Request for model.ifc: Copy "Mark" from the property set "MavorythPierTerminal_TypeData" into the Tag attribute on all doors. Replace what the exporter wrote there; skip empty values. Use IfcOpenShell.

First a look at what the model holds.

```python
import ifcopenshell
import ifcopenshell.util.element

model = ifcopenshell.open("model.ifc")
print(model.schema)
doors = model.by_type("IfcDoor")
print(len(doors), "doors")
for e in doors[:8]:
    source = ifcopenshell.util.element.get_pset(e, "MavorythPierTerminal_TypeData", "Mark")
    target = e.Tag
    print(e.id(), repr(source), repr(target), sep=" | ")
```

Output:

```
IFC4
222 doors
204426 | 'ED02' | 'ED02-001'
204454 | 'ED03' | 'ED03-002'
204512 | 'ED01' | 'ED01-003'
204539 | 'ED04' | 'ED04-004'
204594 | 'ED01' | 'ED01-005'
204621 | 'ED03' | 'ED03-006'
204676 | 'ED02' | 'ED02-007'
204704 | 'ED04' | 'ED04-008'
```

```python
import ifcopenshell
import ifcopenshell.util.element

model = ifcopenshell.open("model.ifc")

count = 0
for e in model.by_type("IfcDoor"):
    value = ifcopenshell.util.element.get_pset(e, "MavorythPierTerminal_TypeData", "Mark")
    current = e.Tag
    if not value or not value.strip() or current == value:
        continue
    e.Tag = value
    count += 1

print(count, "doors updated")

model.write("model-out.ifc")
```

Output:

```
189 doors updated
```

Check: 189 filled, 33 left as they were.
